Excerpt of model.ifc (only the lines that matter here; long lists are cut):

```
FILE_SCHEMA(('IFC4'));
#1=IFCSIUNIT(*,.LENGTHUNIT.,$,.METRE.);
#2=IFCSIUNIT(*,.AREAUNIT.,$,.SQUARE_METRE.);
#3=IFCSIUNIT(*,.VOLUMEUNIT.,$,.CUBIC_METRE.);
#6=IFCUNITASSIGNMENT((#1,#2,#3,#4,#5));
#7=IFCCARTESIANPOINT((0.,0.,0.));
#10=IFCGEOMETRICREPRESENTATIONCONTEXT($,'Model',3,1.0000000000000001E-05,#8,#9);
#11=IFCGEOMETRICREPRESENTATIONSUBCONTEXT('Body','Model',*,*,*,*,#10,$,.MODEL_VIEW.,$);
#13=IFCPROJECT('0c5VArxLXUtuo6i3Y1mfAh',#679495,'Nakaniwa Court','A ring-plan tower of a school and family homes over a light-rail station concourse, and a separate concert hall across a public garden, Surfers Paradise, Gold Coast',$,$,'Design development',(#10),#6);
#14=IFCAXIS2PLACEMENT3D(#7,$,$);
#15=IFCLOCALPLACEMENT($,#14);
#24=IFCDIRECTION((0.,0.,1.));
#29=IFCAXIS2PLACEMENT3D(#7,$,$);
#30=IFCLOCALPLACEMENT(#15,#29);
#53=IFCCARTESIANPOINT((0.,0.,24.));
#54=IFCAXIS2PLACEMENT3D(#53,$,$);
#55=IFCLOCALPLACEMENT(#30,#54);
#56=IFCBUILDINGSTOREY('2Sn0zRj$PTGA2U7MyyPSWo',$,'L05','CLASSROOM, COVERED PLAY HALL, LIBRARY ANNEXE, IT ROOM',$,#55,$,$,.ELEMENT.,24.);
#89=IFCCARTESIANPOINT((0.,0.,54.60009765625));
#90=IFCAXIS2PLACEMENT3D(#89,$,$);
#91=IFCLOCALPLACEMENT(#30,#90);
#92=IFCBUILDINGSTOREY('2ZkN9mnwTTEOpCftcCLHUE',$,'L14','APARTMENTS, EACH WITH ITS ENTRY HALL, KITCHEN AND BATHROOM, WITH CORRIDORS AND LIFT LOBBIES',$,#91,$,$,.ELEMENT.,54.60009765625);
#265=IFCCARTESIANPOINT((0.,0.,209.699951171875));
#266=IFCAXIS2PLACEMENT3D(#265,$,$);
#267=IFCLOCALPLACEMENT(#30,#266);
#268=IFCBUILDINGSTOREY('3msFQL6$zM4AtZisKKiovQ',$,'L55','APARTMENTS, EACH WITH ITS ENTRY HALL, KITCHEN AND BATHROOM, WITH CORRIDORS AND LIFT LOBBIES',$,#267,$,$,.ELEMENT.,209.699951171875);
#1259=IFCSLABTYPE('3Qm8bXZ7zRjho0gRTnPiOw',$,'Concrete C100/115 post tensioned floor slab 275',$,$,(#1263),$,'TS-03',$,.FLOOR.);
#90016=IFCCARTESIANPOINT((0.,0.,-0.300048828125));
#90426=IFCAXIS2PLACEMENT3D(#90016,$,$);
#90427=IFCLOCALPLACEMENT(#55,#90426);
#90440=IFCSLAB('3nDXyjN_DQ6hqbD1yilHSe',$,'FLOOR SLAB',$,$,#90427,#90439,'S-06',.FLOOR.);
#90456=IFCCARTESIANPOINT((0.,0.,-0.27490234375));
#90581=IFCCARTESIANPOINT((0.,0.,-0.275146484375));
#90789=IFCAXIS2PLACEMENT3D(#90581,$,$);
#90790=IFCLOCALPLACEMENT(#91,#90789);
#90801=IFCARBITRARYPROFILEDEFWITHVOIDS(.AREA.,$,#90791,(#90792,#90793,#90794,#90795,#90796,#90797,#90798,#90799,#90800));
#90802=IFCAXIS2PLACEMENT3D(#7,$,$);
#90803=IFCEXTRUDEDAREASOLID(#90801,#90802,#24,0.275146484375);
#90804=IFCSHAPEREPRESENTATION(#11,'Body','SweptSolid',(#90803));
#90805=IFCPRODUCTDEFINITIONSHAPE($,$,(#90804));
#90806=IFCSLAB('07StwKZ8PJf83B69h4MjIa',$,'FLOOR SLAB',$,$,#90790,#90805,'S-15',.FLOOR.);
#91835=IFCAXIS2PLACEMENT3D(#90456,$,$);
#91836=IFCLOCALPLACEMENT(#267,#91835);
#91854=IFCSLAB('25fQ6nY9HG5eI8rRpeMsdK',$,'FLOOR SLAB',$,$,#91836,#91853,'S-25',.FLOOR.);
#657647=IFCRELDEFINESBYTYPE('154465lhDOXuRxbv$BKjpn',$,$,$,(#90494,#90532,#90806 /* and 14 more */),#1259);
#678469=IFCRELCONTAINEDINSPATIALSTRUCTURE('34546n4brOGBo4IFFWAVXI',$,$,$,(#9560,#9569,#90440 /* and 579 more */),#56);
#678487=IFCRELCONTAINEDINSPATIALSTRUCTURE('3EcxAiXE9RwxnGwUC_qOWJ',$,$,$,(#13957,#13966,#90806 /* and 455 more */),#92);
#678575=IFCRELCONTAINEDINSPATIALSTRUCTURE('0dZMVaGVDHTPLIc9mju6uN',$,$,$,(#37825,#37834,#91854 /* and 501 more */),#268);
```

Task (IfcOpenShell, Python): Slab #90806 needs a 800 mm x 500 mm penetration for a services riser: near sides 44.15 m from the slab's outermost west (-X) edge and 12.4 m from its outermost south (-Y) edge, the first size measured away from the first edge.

```python
import numpy as np
import ifcopenshell
import ifcopenshell.api.feature
import ifcopenshell.api.geometry
import ifcopenshell.api.root
import ifcopenshell.geom
import ifcopenshell.util.placement
import ifcopenshell.util.representation
import ifcopenshell.util.shape
import ifcopenshell.util.unit

model = ifcopenshell.open("model.ifc")
unit_scale = ifcopenshell.util.unit.calculate_unit_scale(model)
settings = ifcopenshell.geom.settings()


def volume(element):
    """Net volume in cubic metres, openings subtracted."""
    shape = ifcopenshell.geom.create_shape(settings, element)
    return ifcopenshell.util.shape.get_volume(shape.geometry)


slab = model.by_guid("07StwKZ8PJf83B69h4MjIa")
before = volume(slab)

# Extent in the slab's own axes, in metres. The edges named are its -X and -Y sides.
slab_shape = ifcopenshell.geom.create_shape(settings, slab)
vertices = ifcopenshell.util.shape.get_vertices(slab_shape.geometry)
x_min, y_min, bottom = vertices.min(axis=0)
top = vertices[:, 2].max()

opening = ifcopenshell.api.root.create_entity(model, ifc_class="IfcOpeningElement", name="Services riser opening", predefined_type="OPENING")
context = ifcopenshell.util.representation.get_context(model, "Model", "Body", "MODEL_VIEW")
width, depth = 0.8, 0.5
outline = [(0.0, 0.0), (width, 0.0), (width, depth), (0.0, depth), (0.0, 0.0)]
# Overshoot both faces by 50 mm so the cut is clean.
shape = ifcopenshell.api.geometry.add_slab_representation(
    model, context=context, depth=top - bottom + 0.1, polyline=outline
)
ifcopenshell.api.geometry.assign_representation(model, product=opening, representation=shape)

matrix = ifcopenshell.util.placement.get_local_placement(slab.ObjectPlacement)
matrix[:, 3] = matrix @ np.append(np.array([x_min + 44.15, y_min + 12.4, bottom - 0.05]) / unit_scale, 1.0)
ifcopenshell.api.geometry.edit_object_placement(model, product=opening, matrix=matrix, is_si=False)
ifcopenshell.api.feature.add_feature(model, feature=opening, element=slab)

after = volume(slab)

print(f"slab volume {before:.3f} -> {after:.3f} m3")

model.write("model_edited.ifc")
```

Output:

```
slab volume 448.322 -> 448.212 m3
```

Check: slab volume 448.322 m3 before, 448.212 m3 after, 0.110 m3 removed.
